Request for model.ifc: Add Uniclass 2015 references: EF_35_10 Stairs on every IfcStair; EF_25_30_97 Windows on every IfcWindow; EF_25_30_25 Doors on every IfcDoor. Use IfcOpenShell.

First a look at what the model holds.

```python
import ifcopenshell

model = ifcopenshell.open("model.ifc")
print(model.schema)
print("classifications:", [c.Name for c in model.by_type("IfcClassification")])
for ifc_class in ("IfcDoor", "IfcRoof", "IfcStair", "IfcWall", "IfcWindow"):
    print(ifc_class, len(model.by_type(ifc_class)))
```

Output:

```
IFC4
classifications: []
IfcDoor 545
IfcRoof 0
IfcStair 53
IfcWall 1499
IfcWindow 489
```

```python
import ifcopenshell
import ifcopenshell.api.classification

model = ifcopenshell.open("model.ifc")

system = ifcopenshell.api.classification.add_classification(model, classification="Uniclass 2015")

codes = {
    "IfcStair": ("EF_35_10", "Stairs"),
    "IfcWindow": ("EF_25_30_97", "Windows"),
    "IfcDoor": ("EF_25_30_25", "Doors"),
}
for ifc_class, (code, name) in codes.items():
    products = model.by_type(ifc_class)
    ifcopenshell.api.classification.add_reference(
        model, products=products, classification=system, identification=code, name=name
    )
    print(code, len(products))

model.write("model_updated.ifc")
```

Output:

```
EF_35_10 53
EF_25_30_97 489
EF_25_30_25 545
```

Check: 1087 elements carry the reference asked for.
